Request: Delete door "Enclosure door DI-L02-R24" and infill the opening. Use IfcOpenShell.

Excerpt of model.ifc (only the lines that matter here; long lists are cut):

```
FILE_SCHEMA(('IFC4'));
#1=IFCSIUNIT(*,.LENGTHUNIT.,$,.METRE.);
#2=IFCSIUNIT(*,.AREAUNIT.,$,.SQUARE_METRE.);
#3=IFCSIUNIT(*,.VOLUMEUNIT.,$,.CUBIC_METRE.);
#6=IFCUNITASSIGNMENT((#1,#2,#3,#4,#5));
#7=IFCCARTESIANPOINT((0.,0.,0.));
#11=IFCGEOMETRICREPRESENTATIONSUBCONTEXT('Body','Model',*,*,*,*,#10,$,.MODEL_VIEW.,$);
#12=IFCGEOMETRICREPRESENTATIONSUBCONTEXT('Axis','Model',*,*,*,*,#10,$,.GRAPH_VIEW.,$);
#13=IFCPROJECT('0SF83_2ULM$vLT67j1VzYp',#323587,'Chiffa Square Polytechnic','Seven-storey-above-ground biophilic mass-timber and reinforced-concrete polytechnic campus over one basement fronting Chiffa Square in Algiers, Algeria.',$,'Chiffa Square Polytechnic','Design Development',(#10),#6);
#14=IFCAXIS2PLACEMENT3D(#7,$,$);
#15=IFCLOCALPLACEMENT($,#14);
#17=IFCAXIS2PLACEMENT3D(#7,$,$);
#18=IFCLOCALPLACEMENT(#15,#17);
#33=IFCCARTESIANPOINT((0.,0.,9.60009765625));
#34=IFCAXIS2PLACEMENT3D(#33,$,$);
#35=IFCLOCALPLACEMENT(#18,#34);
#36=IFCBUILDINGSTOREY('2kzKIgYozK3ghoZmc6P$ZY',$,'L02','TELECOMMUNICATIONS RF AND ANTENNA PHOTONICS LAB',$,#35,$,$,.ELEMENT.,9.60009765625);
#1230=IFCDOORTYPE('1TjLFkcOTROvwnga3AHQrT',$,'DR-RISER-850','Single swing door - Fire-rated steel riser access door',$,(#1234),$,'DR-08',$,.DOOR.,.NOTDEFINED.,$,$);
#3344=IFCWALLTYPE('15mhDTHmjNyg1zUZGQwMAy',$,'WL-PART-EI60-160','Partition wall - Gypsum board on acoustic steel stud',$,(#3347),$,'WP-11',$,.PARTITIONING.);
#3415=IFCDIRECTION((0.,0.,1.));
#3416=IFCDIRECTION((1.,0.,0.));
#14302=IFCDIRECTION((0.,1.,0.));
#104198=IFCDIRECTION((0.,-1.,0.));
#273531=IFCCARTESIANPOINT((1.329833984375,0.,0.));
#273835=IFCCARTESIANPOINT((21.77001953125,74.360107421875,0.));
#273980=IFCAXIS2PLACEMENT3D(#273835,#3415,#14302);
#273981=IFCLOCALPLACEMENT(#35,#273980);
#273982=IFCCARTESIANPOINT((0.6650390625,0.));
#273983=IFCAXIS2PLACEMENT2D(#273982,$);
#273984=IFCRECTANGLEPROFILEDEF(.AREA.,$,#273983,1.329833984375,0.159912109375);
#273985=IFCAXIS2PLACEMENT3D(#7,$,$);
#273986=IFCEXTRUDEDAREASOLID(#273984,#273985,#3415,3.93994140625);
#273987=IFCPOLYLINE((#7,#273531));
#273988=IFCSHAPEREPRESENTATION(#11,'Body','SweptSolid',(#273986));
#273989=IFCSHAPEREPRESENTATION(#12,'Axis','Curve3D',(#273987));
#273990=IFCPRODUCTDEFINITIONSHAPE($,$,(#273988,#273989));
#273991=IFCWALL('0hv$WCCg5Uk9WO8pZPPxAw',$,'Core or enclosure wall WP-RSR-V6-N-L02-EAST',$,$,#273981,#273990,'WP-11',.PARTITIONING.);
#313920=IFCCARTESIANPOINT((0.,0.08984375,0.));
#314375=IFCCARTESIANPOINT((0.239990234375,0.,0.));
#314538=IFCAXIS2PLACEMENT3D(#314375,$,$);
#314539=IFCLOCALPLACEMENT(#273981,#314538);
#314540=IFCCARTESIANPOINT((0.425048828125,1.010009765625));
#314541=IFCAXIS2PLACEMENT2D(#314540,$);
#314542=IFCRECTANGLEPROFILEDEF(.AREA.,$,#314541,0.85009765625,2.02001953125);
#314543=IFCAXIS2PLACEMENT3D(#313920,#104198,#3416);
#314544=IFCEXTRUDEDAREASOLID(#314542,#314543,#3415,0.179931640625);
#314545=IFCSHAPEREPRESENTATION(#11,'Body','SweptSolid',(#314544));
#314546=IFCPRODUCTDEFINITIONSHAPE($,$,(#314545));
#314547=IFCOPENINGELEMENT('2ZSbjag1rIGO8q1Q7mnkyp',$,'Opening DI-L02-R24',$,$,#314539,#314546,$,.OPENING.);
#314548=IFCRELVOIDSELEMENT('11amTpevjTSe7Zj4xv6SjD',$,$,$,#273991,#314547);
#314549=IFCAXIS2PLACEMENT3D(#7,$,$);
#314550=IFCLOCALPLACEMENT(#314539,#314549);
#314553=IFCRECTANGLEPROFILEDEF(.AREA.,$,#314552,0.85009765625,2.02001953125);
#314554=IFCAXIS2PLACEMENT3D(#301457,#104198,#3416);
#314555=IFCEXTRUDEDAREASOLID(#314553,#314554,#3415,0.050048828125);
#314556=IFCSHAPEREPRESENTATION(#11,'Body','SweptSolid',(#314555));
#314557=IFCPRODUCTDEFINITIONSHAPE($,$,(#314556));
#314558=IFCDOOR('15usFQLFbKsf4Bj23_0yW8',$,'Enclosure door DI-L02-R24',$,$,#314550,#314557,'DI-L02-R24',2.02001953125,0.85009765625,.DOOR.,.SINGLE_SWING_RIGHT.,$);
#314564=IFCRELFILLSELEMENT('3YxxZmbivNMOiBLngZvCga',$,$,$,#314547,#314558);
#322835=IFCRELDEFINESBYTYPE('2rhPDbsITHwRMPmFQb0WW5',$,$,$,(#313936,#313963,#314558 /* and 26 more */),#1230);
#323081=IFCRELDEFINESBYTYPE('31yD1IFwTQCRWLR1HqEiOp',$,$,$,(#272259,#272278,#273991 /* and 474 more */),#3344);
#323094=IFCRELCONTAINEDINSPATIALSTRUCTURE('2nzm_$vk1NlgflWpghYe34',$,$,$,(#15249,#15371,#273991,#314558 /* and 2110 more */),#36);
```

```python
import ifcopenshell
import ifcopenshell.api.feature
import ifcopenshell.api.root
import ifcopenshell.geom
import ifcopenshell.util.shape

model = ifcopenshell.open("model.ifc")
settings = ifcopenshell.geom.settings()


def volume(element):
    """Net volume in cubic metres, openings subtracted."""
    shape = ifcopenshell.geom.create_shape(settings, element)
    return ifcopenshell.util.shape.get_volume(shape.geometry)


door = model.by_id(314558)
opening = door.FillsVoids[0].RelatingOpeningElement
wall = opening.VoidsElements[0].RelatingBuildingElement
before = volume(wall)

ifcopenshell.api.root.remove_product(model, product=door)
ifcopenshell.api.feature.remove_feature(model, feature=opening)

after = volume(wall)

print(f"wall volume {before:.3f} -> {after:.3f} m3")

model.write("model_edited.ifc")
```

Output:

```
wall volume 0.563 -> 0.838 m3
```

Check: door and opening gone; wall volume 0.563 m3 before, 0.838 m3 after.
